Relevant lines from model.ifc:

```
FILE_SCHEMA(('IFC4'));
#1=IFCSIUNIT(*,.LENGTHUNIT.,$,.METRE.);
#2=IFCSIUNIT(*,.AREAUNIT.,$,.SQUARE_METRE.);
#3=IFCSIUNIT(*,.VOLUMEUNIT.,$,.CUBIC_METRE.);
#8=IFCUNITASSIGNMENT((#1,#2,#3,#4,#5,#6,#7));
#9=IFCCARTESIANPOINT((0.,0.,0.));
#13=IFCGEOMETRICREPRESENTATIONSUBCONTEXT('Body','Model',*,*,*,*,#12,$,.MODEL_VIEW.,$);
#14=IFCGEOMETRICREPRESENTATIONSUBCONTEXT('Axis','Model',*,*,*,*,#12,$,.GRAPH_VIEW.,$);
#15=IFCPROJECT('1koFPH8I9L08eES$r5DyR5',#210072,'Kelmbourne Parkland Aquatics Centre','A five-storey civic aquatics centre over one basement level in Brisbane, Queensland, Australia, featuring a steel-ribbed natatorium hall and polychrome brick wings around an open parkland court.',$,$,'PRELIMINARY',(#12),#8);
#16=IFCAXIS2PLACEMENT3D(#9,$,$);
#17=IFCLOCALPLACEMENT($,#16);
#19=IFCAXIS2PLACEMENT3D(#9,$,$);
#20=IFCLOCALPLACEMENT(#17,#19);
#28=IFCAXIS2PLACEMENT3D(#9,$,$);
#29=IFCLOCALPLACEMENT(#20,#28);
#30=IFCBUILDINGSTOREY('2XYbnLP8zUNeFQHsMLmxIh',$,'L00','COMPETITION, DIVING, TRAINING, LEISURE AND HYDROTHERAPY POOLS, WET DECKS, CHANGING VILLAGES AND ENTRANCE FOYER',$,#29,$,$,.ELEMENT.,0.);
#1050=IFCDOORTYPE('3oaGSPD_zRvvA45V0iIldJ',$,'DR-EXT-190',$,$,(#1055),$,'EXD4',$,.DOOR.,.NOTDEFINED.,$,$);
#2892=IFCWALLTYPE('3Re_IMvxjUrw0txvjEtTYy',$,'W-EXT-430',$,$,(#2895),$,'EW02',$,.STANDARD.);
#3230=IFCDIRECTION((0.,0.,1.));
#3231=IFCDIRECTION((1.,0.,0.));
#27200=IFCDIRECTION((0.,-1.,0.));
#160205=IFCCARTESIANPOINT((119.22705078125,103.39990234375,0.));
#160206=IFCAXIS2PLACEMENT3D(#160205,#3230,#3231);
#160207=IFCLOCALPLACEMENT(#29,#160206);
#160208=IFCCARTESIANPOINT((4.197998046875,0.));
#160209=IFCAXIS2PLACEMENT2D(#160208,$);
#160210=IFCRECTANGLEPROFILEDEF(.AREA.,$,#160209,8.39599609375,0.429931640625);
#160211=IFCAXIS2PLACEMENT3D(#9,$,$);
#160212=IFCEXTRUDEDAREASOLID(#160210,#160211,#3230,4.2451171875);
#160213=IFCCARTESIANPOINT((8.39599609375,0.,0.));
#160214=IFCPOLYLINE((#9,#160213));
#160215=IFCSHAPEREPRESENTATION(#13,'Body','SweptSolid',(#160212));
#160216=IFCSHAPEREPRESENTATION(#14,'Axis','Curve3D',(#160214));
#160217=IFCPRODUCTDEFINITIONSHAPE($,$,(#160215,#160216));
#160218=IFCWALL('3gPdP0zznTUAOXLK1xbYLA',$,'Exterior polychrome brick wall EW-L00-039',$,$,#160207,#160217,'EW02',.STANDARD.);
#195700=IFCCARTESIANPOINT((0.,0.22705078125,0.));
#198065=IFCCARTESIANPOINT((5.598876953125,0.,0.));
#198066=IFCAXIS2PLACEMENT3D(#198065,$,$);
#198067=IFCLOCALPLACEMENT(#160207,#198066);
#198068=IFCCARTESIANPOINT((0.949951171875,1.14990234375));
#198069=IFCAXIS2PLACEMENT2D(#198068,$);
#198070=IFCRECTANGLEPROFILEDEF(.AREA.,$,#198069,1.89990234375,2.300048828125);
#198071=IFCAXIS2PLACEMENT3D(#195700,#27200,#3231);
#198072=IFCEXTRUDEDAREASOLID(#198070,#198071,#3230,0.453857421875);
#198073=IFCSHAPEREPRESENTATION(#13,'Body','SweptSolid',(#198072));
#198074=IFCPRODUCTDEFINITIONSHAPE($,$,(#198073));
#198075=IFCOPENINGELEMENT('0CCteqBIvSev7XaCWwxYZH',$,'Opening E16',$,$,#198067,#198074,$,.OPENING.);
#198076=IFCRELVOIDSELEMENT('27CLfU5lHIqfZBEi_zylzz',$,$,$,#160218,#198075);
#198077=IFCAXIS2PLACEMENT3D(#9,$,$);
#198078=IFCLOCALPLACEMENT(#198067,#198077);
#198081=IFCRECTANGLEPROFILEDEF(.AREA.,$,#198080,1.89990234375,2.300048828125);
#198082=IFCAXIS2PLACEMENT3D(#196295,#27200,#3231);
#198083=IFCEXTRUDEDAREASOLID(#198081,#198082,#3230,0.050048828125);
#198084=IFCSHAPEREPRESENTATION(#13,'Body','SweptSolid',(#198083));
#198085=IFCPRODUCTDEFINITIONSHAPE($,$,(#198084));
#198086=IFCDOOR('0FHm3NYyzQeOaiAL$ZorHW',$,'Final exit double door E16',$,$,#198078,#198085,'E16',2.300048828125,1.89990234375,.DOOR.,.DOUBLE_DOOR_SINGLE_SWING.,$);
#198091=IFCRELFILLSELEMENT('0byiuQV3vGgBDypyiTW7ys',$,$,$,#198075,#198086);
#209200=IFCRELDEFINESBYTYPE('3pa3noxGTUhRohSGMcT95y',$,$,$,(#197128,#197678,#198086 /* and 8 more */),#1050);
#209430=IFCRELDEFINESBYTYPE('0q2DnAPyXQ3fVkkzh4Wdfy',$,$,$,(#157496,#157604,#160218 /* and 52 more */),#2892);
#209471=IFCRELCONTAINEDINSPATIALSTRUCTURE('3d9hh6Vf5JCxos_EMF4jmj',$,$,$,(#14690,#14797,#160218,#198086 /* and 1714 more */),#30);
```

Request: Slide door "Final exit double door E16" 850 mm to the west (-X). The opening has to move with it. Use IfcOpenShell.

```python
import ifcopenshell
import ifcopenshell.api.geometry
import ifcopenshell.util.placement
import ifcopenshell.util.unit

model = ifcopenshell.open("model.ifc")
unit_scale = ifcopenshell.util.unit.calculate_unit_scale(model)

door = model.by_id(198086)
opening = door.FillsVoids[0].RelatingOpeningElement
wall = opening.VoidsElements[0].RelatingBuildingElement

wall_matrix = ifcopenshell.util.placement.get_local_placement(wall.ObjectPlacement)
shift = wall_matrix[:3, 0] * -0.85 / unit_scale
before = ifcopenshell.util.placement.get_local_placement(door.ObjectPlacement)[:3, 3].copy()

# The door is placed relative to its opening, so it follows when the opening moves.
matrix = ifcopenshell.util.placement.get_local_placement(opening.ObjectPlacement)
matrix[:3, 3] += shift
ifcopenshell.api.geometry.edit_object_placement(
    model, product=opening, matrix=matrix, is_si=False, should_transform_children=True
)

after = ifcopenshell.util.placement.get_local_placement(door.ObjectPlacement)[:3, 3]
print("door moved by", (after - before).round(3) + 0.0)

model.write("model_edited.ifc")
```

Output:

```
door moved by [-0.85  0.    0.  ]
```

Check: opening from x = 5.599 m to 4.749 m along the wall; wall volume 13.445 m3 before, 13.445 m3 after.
